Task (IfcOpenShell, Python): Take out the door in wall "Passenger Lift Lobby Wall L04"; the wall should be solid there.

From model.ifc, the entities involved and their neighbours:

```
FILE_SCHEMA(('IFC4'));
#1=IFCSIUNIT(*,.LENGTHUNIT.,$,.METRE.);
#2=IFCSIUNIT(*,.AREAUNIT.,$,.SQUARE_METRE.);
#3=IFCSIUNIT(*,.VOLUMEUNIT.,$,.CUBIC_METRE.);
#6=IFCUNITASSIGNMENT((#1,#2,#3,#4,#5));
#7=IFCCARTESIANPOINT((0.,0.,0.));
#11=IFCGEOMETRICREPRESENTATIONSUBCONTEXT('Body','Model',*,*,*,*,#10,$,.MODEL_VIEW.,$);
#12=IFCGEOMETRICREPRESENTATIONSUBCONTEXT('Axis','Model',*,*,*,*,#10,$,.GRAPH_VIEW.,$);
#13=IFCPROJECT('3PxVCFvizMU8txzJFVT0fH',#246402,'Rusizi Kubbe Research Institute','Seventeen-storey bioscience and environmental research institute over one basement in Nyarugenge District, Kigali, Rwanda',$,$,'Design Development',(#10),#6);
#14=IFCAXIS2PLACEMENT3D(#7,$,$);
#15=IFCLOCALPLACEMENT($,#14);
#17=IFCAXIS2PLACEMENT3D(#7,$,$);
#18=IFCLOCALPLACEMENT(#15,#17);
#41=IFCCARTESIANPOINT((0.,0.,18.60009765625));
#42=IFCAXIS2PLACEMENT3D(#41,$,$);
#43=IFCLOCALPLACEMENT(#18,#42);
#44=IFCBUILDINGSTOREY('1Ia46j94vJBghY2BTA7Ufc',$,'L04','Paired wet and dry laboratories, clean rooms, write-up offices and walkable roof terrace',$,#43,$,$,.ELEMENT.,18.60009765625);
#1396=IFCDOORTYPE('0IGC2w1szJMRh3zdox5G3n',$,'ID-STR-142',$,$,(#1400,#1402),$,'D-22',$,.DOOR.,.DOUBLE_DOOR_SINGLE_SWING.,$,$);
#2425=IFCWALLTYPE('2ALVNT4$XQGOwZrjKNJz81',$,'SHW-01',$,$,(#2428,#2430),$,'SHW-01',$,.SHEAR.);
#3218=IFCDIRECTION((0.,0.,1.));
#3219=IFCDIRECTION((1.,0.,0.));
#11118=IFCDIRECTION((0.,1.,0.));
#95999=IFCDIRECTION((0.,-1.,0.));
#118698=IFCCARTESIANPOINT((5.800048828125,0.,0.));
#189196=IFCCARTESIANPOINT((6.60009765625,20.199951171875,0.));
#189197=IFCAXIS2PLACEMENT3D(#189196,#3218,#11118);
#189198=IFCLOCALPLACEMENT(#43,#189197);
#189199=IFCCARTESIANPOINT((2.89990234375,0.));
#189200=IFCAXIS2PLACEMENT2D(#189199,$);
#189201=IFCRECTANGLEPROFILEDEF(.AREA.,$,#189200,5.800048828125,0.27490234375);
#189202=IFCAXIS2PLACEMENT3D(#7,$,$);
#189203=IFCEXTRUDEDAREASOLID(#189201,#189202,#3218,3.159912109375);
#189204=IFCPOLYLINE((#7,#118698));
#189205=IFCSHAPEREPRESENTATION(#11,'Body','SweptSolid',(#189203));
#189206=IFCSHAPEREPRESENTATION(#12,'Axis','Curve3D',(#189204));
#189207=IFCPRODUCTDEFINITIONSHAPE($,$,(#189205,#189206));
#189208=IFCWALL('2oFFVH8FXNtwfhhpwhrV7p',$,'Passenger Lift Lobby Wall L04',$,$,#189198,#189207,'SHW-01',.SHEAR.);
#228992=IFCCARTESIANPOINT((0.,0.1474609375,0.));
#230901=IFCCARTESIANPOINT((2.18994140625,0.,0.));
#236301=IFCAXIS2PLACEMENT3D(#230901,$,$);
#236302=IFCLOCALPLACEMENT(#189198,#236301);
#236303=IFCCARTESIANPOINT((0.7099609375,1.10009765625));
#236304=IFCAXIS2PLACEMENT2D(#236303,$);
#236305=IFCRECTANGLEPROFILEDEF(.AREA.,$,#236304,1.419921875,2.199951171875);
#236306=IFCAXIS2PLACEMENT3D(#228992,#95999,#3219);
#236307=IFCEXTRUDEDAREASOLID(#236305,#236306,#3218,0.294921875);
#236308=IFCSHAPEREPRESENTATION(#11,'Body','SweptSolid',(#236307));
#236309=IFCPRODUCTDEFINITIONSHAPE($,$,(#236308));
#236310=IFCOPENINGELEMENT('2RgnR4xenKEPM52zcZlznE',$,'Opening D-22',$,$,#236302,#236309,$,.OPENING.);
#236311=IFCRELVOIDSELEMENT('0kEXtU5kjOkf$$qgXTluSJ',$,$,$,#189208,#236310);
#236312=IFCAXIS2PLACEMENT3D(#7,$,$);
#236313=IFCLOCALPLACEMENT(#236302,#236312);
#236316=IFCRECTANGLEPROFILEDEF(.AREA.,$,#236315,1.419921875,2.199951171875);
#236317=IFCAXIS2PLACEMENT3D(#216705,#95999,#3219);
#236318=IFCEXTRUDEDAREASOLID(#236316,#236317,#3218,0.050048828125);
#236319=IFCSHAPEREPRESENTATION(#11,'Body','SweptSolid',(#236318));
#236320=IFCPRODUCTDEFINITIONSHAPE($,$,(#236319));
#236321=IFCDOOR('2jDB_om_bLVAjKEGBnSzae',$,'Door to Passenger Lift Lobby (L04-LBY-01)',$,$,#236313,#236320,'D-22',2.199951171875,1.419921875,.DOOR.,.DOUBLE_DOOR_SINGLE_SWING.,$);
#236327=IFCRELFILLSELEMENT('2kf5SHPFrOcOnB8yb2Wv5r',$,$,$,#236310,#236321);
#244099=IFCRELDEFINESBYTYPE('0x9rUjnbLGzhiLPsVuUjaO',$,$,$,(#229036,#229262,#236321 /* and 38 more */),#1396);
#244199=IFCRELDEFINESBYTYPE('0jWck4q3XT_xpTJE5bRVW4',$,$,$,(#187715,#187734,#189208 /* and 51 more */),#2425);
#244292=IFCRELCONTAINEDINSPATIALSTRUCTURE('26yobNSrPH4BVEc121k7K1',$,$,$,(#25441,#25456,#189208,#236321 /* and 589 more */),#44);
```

```python
import ifcopenshell
import ifcopenshell.api.feature
import ifcopenshell.api.root
import ifcopenshell.geom
import ifcopenshell.util.shape

model = ifcopenshell.open("model.ifc")
settings = ifcopenshell.geom.settings()


def volume(element):
    """Net volume in cubic metres, openings subtracted."""
    shape = ifcopenshell.geom.create_shape(settings, element)
    return ifcopenshell.util.shape.get_volume(shape.geometry)


door = model.by_id(236321)
opening = door.FillsVoids[0].RelatingOpeningElement
wall = opening.VoidsElements[0].RelatingBuildingElement
before = volume(wall)

ifcopenshell.api.root.remove_product(model, product=door)
ifcopenshell.api.feature.remove_feature(model, feature=opening)

after = volume(wall)

print(f"wall volume {before:.3f} -> {after:.3f} m3")

model.write("model_v2.ifc")
```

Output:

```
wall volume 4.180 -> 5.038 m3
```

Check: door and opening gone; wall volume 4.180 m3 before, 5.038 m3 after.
